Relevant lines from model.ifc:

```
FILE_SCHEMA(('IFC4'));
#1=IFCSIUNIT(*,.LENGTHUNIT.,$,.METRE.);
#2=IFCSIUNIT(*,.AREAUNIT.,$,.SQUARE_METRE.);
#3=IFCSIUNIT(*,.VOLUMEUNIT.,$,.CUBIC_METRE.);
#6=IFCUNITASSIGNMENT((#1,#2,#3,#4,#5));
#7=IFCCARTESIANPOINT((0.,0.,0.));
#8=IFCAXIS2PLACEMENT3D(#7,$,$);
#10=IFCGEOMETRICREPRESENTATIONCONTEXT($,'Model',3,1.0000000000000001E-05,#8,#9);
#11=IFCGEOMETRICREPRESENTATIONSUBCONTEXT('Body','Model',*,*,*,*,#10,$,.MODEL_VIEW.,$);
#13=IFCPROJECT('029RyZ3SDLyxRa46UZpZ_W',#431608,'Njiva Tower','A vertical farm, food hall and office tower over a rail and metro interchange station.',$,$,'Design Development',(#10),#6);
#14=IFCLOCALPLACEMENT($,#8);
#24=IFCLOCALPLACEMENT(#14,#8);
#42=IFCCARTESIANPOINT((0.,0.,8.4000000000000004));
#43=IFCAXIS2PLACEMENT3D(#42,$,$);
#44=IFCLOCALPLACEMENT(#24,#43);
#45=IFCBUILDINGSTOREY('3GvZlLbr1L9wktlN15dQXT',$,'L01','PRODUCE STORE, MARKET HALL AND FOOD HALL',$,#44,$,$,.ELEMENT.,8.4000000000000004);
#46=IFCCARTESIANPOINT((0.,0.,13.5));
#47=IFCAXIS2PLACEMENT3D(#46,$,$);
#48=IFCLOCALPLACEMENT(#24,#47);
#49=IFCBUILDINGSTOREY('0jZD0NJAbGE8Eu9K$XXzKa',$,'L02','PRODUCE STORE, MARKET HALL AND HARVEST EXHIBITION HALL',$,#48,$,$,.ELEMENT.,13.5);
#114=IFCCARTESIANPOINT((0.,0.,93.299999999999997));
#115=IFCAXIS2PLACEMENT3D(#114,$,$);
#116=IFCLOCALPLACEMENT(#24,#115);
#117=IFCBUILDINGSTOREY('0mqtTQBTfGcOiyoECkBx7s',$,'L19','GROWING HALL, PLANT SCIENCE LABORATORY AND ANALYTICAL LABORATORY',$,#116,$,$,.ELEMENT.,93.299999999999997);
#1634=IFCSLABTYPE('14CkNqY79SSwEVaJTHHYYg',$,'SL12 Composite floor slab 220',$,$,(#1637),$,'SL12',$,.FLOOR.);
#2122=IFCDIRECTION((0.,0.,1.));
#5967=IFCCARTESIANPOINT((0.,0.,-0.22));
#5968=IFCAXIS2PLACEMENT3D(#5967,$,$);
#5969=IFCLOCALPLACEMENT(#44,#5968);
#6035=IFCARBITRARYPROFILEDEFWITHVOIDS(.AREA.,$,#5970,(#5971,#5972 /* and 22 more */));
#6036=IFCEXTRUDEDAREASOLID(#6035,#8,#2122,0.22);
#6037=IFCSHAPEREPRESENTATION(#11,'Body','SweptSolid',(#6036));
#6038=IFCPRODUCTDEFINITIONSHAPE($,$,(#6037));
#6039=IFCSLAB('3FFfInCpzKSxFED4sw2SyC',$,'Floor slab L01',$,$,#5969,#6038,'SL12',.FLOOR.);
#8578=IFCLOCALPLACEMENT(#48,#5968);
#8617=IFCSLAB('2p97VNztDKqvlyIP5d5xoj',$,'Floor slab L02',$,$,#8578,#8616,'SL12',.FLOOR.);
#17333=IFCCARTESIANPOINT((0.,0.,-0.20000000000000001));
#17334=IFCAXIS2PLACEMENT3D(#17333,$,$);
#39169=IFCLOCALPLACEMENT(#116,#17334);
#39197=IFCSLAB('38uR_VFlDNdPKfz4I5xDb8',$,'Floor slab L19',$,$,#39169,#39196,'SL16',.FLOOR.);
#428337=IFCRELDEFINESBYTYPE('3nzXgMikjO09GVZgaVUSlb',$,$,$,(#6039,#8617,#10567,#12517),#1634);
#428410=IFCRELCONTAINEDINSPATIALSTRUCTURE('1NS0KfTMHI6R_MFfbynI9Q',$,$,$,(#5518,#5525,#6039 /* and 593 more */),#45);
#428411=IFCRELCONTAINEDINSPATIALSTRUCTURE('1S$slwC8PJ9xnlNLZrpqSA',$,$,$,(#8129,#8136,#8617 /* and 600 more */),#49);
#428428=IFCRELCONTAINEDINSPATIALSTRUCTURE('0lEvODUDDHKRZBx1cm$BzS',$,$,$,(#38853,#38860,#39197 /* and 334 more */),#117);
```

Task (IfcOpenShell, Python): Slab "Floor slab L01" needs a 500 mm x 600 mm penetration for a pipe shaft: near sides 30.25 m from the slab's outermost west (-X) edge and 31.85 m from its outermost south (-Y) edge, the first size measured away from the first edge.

```python
import numpy as np
import ifcopenshell
import ifcopenshell.api.feature
import ifcopenshell.api.geometry
import ifcopenshell.api.root
import ifcopenshell.geom
import ifcopenshell.util.placement
import ifcopenshell.util.representation
import ifcopenshell.util.shape
import ifcopenshell.util.unit

model = ifcopenshell.open("model.ifc")
unit_scale = ifcopenshell.util.unit.calculate_unit_scale(model)
settings = ifcopenshell.geom.settings()


def volume(element):
    """Net volume in cubic metres, openings subtracted."""
    shape = ifcopenshell.geom.create_shape(settings, element)
    return ifcopenshell.util.shape.get_volume(shape.geometry)


slab = model.by_guid("3FFfInCpzKSxFED4sw2SyC")
before = volume(slab)

# Extent in the slab's own axes, in metres. The edges named are its -X and -Y sides.
slab_shape = ifcopenshell.geom.create_shape(settings, slab)
vertices = ifcopenshell.util.shape.get_vertices(slab_shape.geometry)
x_min, y_min, bottom = vertices.min(axis=0)
top = vertices[:, 2].max()

opening = ifcopenshell.api.root.create_entity(model, ifc_class="IfcOpeningElement", name="Pipe shaft opening", predefined_type="OPENING")
context = ifcopenshell.util.representation.get_context(model, "Model", "Body", "MODEL_VIEW")
width, depth = 0.5, 0.6
outline = [(0.0, 0.0), (width, 0.0), (width, depth), (0.0, depth), (0.0, 0.0)]
# Overshoot both faces by 50 mm so the cut is clean.
shape = ifcopenshell.api.geometry.add_slab_representation(
    model, context=context, depth=top - bottom + 0.1, polyline=outline
)
ifcopenshell.api.geometry.assign_representation(model, product=opening, representation=shape)

matrix = ifcopenshell.util.placement.get_local_placement(slab.ObjectPlacement)
matrix[:, 3] = matrix @ np.append(np.array([x_min + 30.25, y_min + 31.85, bottom - 0.05]) / unit_scale, 1.0)
ifcopenshell.api.geometry.edit_object_placement(model, product=opening, matrix=matrix, is_si=False)
ifcopenshell.api.feature.add_feature(model, feature=opening, element=slab)

after = volume(slab)

print(f"slab volume {before:.3f} -> {after:.3f} m3")

model.write("model_v2.ifc")
```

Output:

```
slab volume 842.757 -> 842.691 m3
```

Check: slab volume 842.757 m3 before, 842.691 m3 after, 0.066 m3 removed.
